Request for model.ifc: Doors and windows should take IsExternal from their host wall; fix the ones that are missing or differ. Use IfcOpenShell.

First a look at what the model holds.

```python
import ifcopenshell
import ifcopenshell.util.element

model = ifcopenshell.open("model.ifc")
print(model.schema)
seen = {}
for e in model.by_type("IfcDoor") + model.by_type("IfcWindow"):
    if not e.FillsVoids:
        continue
    host = e.FillsVoids[0].RelatingOpeningElement.VoidsElements[0].RelatingBuildingElement
    own = ifcopenshell.util.element.get_pset(e, f"Pset_{e.is_a()[3:].removesuffix('StandardCase')}Common", "IsExternal")
    wall = ifcopenshell.util.element.get_pset(host, "Pset_WallCommon", "IsExternal")
    seen[e.is_a(), own, wall] = seen.get((e.is_a(), own, wall), 0) + 1
for (cls, own, wall), count in sorted(seen.items(), key=str):
    print(count, cls, "IsExternal:", own, "| host wall:", wall)
```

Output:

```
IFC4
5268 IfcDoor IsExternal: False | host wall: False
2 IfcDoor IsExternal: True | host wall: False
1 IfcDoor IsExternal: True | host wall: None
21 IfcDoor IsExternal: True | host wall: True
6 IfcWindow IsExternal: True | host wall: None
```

```python
import ifcopenshell
import ifcopenshell.api.pset
import ifcopenshell.util.element

model = ifcopenshell.open("model.ifc")

count = 0
for ifc_class, pset_name in (("IfcDoor", "Pset_DoorCommon"), ("IfcWindow", "Pset_WindowCommon")):
    for e in model.by_type(ifc_class):
        if not e.FillsVoids:
            continue
        host = e.FillsVoids[0].RelatingOpeningElement.VoidsElements[0].RelatingBuildingElement
        external = ifcopenshell.util.element.get_pset(host, "Pset_WallCommon", "IsExternal")
        if external is None or ifcopenshell.util.element.get_pset(e, pset_name, "IsExternal") == external:
            continue
        found = ifcopenshell.util.element.get_pset(e, pset_name, should_inherit=False)
        if found:
            pset = model.by_id(found["id"])
            if len(ifcopenshell.util.element.get_elements_by_pset(pset)) > 1:
                pset = ifcopenshell.api.pset.unshare_pset(model, products=[e], pset=pset)[0]
        else:
            pset = ifcopenshell.api.pset.add_pset(model, product=e, name=pset_name)
        ifcopenshell.api.pset.edit_pset(model, pset=pset, properties={"IsExternal": external})
        count += 1

print(count, "updated")

model.write("model_rev.ifc")
```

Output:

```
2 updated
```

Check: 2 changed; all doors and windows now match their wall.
